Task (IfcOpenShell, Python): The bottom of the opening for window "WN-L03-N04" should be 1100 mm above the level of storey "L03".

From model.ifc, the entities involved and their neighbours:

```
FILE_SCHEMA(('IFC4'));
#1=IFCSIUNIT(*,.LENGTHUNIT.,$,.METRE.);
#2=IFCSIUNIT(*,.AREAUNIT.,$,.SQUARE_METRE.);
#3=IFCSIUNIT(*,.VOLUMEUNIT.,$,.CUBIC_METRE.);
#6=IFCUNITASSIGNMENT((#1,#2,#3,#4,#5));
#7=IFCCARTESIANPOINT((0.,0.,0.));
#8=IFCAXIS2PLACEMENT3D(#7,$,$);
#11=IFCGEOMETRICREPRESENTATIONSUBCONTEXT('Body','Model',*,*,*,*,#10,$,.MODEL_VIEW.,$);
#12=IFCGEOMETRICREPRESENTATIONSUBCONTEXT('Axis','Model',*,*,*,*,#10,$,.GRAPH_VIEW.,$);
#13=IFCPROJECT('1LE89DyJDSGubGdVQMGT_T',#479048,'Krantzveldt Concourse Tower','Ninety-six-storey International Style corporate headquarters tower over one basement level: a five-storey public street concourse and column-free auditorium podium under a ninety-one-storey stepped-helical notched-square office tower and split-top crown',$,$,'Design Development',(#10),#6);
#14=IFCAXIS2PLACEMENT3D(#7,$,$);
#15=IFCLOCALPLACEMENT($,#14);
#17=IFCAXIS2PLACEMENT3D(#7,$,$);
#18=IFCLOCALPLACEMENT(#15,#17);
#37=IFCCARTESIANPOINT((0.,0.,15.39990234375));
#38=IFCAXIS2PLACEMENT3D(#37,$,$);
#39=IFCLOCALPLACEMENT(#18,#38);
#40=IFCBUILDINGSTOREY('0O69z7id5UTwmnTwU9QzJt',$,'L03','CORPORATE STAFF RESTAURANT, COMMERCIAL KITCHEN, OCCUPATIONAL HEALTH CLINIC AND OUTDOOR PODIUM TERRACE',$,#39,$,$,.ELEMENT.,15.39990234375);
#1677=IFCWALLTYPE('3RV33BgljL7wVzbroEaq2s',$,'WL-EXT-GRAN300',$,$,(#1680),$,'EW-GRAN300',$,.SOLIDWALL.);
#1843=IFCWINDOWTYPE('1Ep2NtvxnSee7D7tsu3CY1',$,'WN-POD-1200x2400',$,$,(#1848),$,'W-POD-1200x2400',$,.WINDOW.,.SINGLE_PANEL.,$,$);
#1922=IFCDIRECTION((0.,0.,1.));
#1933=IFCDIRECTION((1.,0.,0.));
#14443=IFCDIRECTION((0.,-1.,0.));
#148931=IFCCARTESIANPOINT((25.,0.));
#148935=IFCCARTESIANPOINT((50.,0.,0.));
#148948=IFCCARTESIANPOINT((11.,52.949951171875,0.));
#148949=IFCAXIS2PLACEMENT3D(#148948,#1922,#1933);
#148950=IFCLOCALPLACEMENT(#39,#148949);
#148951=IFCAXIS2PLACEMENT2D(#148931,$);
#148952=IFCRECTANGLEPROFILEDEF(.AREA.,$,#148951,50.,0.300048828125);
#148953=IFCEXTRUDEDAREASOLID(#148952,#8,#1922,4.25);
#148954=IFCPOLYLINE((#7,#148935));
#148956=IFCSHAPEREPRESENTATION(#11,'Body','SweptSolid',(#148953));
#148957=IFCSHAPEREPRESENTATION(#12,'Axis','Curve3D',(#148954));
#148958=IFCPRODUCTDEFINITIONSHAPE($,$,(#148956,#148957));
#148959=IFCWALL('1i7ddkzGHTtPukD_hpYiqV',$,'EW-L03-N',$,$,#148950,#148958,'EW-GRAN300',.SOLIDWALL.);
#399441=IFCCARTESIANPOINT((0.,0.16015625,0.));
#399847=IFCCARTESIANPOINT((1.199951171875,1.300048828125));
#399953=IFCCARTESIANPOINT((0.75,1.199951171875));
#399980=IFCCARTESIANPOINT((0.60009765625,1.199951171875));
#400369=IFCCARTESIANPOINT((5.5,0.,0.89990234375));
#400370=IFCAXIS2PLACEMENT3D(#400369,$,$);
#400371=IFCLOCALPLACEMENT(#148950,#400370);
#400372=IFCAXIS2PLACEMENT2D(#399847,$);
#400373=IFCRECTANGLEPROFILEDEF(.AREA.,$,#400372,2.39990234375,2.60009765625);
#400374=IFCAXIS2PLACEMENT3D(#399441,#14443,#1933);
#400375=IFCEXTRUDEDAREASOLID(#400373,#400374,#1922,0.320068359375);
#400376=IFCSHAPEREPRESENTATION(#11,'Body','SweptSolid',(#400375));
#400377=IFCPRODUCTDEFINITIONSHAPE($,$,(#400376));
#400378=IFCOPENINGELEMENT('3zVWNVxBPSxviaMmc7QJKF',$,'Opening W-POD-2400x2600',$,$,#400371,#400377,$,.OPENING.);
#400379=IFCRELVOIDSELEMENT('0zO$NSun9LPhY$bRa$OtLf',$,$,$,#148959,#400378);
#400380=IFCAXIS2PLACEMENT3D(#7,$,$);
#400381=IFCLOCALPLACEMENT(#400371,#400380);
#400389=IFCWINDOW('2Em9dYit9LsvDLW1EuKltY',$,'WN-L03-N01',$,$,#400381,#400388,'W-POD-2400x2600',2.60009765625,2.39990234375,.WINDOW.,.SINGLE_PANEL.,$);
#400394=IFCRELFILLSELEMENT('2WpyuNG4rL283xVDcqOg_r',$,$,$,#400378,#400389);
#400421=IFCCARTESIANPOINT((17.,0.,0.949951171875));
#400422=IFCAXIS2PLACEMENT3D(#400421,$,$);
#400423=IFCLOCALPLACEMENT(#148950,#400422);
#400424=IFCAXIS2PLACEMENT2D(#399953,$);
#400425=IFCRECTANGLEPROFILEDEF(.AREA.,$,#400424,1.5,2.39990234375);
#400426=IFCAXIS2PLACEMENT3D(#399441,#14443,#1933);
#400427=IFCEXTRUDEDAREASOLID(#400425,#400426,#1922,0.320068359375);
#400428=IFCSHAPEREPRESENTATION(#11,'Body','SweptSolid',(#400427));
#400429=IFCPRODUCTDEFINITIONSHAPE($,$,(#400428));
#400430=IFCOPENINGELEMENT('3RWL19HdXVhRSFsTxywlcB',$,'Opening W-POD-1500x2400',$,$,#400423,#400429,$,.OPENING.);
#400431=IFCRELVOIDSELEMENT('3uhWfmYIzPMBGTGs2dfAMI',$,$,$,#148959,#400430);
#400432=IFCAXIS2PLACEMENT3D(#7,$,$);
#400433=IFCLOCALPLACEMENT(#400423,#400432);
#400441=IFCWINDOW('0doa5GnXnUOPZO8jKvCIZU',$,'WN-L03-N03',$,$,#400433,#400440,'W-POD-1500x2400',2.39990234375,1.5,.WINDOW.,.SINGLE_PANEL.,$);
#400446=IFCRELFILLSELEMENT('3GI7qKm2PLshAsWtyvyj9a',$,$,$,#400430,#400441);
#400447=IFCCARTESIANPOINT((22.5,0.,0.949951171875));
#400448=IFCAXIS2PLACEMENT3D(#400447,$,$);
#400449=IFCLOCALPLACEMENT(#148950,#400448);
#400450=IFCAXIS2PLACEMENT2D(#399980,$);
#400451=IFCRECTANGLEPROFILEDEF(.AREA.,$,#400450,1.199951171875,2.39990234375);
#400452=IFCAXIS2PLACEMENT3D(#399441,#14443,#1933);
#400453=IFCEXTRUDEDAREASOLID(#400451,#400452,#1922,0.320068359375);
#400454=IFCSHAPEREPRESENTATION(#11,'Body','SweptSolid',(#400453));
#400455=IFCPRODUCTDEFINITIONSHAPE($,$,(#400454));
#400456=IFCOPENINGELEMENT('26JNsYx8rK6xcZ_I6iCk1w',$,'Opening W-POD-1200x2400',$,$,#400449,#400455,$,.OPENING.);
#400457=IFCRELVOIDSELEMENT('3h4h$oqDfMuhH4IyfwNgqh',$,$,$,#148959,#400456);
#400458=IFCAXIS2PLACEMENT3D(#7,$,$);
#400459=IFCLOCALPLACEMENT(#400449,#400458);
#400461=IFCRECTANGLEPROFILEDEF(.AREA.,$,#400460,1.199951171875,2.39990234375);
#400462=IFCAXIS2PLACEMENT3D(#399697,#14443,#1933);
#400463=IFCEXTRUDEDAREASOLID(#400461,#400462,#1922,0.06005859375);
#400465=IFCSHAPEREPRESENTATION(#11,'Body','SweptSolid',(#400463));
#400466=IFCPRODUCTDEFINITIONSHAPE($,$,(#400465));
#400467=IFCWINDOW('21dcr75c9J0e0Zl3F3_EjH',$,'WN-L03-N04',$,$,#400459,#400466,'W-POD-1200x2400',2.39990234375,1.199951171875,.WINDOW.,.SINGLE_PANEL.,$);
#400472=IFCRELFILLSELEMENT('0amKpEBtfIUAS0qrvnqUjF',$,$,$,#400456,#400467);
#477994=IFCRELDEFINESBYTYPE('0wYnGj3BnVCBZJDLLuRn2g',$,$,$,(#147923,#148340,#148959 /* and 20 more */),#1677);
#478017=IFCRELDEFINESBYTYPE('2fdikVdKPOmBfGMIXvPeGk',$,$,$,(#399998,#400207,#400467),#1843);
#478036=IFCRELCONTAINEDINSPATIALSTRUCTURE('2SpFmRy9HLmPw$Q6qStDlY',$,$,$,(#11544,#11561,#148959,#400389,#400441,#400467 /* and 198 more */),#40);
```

```python
import numpy as np
import ifcopenshell
import ifcopenshell.api.geometry
import ifcopenshell.geom
import ifcopenshell.util.element
import ifcopenshell.util.placement
import ifcopenshell.util.shape
import ifcopenshell.util.unit

model = ifcopenshell.open("model.ifc")
unit_scale = ifcopenshell.util.unit.calculate_unit_scale(model)

window = model.by_guid("21dcr75c9J0e0Zl3F3_EjH")
opening = window.FillsVoids[0].RelatingOpeningElement
storey = ifcopenshell.util.element.get_container(window, ifc_class="IfcBuildingStorey")
level = ifcopenshell.util.placement.get_local_placement(storey.ObjectPlacement)[2, 3]

# The opening's origin need not be at the sill, so measure its lowest point.
shape = ifcopenshell.geom.create_shape(ifcopenshell.geom.settings(), opening)
bottom = ifcopenshell.util.shape.get_shape_bottom_elevation(shape, shape.geometry) / unit_scale
dz = level + 1.1 / unit_scale - bottom

shift = np.array([0.0, 0.0, dz])
# The window is placed relative to its opening, so it follows when the opening moves.
matrix = ifcopenshell.util.placement.get_local_placement(opening.ObjectPlacement)
matrix[:3, 3] += shift
ifcopenshell.api.geometry.edit_object_placement(
    model, product=opening, matrix=matrix, is_si=False, should_transform_children=True
)

print(f"moved by {dz * unit_scale:+.3f} m")

model.write("model-out.ifc")
```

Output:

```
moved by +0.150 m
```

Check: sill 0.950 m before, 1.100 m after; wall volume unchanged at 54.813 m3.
